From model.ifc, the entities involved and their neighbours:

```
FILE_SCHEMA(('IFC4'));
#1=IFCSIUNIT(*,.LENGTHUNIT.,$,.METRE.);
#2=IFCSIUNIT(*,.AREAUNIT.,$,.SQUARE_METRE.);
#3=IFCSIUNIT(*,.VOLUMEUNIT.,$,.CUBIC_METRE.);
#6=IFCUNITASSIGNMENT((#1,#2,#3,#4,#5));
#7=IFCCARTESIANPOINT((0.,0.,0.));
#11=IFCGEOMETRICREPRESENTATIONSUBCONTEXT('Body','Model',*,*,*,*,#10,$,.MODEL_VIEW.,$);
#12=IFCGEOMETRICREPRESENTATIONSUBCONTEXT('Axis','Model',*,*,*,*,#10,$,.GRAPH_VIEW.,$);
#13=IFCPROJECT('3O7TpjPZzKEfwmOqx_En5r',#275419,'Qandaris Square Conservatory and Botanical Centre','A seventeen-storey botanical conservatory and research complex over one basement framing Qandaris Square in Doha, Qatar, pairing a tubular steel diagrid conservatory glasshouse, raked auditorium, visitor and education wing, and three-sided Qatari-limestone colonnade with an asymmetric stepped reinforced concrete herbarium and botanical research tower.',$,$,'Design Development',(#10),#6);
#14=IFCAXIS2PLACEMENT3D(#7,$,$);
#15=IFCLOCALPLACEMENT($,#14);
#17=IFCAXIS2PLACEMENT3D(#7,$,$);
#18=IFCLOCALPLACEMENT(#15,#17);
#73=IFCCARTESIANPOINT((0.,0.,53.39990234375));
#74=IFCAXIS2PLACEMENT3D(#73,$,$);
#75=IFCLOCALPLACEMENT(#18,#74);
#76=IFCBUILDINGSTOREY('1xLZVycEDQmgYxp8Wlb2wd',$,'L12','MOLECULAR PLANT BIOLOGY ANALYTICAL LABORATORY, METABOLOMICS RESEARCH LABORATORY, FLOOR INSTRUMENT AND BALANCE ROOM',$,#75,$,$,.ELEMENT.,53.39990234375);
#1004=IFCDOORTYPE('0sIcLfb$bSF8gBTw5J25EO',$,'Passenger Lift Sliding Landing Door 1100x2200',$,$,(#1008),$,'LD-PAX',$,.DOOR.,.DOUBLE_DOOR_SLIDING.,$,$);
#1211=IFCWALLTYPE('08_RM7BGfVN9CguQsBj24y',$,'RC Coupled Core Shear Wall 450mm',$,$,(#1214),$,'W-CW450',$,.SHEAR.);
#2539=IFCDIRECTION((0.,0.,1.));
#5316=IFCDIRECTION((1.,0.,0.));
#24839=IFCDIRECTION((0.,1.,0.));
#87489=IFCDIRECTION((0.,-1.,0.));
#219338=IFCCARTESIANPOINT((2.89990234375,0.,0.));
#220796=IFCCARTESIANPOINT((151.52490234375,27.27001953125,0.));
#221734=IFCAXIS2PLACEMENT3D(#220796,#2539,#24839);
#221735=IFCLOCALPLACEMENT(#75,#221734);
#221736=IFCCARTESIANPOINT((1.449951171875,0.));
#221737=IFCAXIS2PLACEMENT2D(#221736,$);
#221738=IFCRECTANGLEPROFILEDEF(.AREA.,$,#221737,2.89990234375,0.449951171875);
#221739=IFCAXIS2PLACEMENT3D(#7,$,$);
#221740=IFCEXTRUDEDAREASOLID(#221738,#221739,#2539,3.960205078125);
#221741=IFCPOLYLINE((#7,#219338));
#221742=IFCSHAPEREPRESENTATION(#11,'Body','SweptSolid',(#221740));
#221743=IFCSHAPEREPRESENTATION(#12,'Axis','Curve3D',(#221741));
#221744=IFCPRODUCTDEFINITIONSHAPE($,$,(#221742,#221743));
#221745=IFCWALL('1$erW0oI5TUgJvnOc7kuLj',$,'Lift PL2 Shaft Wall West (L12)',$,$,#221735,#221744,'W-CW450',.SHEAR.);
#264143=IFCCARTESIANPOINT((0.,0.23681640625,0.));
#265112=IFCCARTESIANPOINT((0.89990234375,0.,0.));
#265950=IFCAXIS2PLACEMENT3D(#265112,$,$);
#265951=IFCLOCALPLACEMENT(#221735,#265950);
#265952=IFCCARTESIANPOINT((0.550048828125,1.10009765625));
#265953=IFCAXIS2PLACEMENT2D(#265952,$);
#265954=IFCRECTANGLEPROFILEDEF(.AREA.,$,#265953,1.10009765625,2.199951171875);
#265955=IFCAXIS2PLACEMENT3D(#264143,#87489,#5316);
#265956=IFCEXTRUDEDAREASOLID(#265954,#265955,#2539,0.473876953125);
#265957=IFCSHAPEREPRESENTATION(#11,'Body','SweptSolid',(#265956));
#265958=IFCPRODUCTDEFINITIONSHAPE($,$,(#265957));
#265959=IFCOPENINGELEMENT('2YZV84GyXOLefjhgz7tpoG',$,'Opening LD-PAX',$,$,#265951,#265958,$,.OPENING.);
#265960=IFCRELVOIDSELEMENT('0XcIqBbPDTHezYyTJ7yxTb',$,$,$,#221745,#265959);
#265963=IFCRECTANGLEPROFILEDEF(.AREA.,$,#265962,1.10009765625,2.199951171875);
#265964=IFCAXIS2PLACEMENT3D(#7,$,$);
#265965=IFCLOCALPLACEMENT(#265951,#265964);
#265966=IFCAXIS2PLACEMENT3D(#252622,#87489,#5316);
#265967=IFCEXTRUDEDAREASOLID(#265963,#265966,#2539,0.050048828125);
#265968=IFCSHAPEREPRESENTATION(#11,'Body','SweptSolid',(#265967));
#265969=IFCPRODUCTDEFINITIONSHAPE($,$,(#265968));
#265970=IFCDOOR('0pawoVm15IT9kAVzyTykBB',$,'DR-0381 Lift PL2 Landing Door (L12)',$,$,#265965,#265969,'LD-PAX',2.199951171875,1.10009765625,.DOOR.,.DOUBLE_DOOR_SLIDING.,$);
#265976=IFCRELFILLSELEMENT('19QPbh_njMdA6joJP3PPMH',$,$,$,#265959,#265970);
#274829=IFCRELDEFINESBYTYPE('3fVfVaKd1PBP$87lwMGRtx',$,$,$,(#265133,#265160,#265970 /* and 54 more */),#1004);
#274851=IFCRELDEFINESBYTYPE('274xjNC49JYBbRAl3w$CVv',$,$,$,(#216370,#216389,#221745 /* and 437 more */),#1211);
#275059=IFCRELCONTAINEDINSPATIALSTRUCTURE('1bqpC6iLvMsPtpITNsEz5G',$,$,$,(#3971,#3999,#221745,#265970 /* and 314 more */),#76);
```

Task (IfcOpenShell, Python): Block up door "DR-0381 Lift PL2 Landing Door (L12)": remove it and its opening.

```python
import ifcopenshell
import ifcopenshell.api.feature
import ifcopenshell.api.root
import ifcopenshell.geom
import ifcopenshell.util.shape

model = ifcopenshell.open("model.ifc")
settings = ifcopenshell.geom.settings()


def volume(element):
    """Net volume in cubic metres, openings subtracted."""
    shape = ifcopenshell.geom.create_shape(settings, element)
    return ifcopenshell.util.shape.get_volume(shape.geometry)


door = model.by_id(265970)
opening = door.FillsVoids[0].RelatingOpeningElement
wall = opening.VoidsElements[0].RelatingBuildingElement
before = volume(wall)

ifcopenshell.api.root.remove_product(model, product=door)
ifcopenshell.api.feature.remove_feature(model, feature=opening)

after = volume(wall)

print(f"wall volume {before:.3f} -> {after:.3f} m3")

model.write("model_v2.ifc")
```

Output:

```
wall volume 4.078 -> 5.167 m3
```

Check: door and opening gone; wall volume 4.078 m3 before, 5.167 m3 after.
